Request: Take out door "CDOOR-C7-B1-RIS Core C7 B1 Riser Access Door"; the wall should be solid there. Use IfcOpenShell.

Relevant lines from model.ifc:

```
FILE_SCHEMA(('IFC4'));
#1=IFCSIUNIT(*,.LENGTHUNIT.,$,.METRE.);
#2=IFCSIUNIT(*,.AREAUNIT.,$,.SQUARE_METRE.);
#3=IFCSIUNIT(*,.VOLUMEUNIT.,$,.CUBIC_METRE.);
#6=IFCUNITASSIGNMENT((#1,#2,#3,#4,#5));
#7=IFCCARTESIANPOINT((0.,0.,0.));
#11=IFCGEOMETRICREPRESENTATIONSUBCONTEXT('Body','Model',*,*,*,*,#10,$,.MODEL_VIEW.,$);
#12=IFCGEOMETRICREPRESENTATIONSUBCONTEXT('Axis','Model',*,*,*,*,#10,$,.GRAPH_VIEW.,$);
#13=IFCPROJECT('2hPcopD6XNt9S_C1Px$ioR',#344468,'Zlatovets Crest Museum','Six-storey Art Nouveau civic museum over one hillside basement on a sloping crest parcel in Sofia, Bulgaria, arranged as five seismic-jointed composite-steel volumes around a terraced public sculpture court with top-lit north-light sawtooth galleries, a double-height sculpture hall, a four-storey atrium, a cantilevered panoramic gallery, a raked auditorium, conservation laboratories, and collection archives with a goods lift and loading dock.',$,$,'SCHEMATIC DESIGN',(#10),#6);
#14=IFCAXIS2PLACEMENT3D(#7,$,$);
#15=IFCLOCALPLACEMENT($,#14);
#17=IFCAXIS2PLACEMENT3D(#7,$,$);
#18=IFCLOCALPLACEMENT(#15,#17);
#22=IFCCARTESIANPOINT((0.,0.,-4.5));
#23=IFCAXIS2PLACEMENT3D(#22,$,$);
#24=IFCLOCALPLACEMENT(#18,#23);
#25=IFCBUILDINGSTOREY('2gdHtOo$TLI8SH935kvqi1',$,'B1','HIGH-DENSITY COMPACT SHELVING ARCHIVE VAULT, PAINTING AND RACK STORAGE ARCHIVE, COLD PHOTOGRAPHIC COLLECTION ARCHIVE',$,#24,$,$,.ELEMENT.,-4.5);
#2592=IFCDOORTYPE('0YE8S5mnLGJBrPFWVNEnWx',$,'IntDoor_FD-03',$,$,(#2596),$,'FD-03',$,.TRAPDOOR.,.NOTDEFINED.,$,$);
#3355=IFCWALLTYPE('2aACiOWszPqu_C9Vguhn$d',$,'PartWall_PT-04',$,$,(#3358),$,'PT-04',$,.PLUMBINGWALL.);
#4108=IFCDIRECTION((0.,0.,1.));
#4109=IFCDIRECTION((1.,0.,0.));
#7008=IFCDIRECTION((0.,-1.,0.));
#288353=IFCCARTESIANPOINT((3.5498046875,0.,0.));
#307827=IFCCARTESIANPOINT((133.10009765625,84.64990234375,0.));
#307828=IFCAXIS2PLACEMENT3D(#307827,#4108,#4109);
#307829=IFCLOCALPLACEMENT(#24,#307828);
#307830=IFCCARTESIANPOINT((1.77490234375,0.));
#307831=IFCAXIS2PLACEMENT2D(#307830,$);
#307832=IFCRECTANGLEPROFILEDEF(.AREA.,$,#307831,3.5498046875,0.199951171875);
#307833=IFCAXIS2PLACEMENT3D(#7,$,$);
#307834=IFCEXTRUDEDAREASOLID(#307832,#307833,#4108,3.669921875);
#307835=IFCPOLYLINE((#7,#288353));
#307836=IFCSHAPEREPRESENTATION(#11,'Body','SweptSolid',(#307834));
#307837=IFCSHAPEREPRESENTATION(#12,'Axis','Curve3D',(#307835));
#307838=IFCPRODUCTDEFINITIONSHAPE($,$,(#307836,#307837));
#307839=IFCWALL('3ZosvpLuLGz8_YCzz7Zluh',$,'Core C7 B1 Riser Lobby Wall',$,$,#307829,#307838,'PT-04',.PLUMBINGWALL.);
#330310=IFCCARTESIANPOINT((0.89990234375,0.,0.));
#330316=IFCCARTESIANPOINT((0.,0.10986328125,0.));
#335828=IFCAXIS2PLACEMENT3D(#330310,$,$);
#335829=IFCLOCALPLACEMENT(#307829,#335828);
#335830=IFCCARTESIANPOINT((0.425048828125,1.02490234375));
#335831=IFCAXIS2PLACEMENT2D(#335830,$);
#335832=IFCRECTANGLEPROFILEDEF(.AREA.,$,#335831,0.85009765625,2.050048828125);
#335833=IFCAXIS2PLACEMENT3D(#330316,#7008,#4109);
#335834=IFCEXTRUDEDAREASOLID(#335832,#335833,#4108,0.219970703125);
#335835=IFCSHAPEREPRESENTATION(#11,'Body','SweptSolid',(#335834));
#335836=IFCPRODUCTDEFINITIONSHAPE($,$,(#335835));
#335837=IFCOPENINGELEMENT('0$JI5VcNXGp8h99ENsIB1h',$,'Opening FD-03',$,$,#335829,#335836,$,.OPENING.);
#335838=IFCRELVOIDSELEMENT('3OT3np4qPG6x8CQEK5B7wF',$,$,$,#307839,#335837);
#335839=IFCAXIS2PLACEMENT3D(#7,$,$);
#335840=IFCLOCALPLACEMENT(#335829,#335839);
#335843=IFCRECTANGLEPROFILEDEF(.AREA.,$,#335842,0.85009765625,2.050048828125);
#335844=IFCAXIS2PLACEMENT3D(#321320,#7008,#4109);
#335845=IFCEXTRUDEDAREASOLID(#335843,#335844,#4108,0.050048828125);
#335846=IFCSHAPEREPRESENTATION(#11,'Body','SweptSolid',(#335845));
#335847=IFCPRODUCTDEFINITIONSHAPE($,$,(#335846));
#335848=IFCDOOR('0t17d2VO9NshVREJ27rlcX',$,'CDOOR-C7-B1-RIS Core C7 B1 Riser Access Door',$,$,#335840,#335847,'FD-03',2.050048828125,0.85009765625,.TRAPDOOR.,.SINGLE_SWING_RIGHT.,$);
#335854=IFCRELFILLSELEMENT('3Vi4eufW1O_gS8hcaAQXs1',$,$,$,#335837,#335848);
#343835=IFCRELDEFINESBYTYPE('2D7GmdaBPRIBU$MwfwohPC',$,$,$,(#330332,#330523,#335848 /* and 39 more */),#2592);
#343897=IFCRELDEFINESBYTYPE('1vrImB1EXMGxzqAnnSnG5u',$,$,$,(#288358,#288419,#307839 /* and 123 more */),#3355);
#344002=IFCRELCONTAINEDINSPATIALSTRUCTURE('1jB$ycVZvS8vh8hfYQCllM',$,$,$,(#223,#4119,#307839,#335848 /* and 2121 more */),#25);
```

```python
import ifcopenshell
import ifcopenshell.api.feature
import ifcopenshell.api.root
import ifcopenshell.geom
import ifcopenshell.util.shape

model = ifcopenshell.open("model.ifc")
settings = ifcopenshell.geom.settings()


def volume(element):
    """Net volume in cubic metres, openings subtracted."""
    shape = ifcopenshell.geom.create_shape(settings, element)
    return ifcopenshell.util.shape.get_volume(shape.geometry)


door = model.by_guid("0t17d2VO9NshVREJ27rlcX")
opening = door.FillsVoids[0].RelatingOpeningElement
wall = opening.VoidsElements[0].RelatingBuildingElement
before = volume(wall)

ifcopenshell.api.root.remove_product(model, product=door)
ifcopenshell.api.feature.remove_feature(model, feature=opening)

after = volume(wall)

print(f"wall volume {before:.3f} -> {after:.3f} m3")

model.write("model_updated.ifc")
```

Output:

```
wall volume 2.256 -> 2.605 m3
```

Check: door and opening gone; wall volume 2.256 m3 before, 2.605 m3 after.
